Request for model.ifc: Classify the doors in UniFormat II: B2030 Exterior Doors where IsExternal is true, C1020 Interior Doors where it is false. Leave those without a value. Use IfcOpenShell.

First a look at what the model holds.

```python
import ifcopenshell
import ifcopenshell.util.element

model = ifcopenshell.open("model.ifc")
print(model.schema)
print("classifications:", [c.Name for c in model.by_type("IfcClassification")])
values = [ifcopenshell.util.element.get_pset(e, "Pset_DoorCommon", "IsExternal") for e in model.by_type("IfcDoor")]
for value in (True, False, None):
    print("IsExternal", value, values.count(value))
```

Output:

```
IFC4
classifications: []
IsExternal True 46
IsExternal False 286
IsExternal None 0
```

```python
import ifcopenshell
import ifcopenshell.api.classification
import ifcopenshell.util.element

model = ifcopenshell.open("model.ifc")

system = ifcopenshell.api.classification.add_classification(model, classification="UniFormat II")

doors = model.by_type("IfcDoor")
external = {e: ifcopenshell.util.element.get_pset(e, "Pset_DoorCommon", "IsExternal") for e in doors}
for flag, code, name in ((True, "B2030", "Exterior Doors"), (False, "C1020", "Interior Doors")):
    products = [e for e in doors if external[e] is flag]
    ifcopenshell.api.classification.add_reference(
        model, products=products, classification=system, identification=code, name=name
    )
    print(code, len(products))

model.write("model-out.ifc")
```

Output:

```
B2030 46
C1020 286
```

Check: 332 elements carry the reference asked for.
